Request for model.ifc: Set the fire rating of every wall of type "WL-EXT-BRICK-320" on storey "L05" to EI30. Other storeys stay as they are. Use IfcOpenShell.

First a look at what the model holds.

```python
import ifcopenshell
import ifcopenshell.util.element

model = ifcopenshell.open("model.ifc")
print(model.schema)
storey = next(s for s in model.by_type("IfcBuildingStorey") if s.Name == "L05")
walls = [e for e in ifcopenshell.util.element.get_decomposition(storey) if e.is_a("IfcWall")]
seen = {}
for e in walls:
    element_type = ifcopenshell.util.element.get_type(e)
    key = (element_type.Name if element_type != e and element_type else None, ifcopenshell.util.element.get_pset(e, "Pset_WallCommon", "FireRating"))
    seen[key] = seen.get(key, 0) + 1
for (name, value), count in sorted(seen.items(), key=str):
    print(count, "x", name, "|", value)
```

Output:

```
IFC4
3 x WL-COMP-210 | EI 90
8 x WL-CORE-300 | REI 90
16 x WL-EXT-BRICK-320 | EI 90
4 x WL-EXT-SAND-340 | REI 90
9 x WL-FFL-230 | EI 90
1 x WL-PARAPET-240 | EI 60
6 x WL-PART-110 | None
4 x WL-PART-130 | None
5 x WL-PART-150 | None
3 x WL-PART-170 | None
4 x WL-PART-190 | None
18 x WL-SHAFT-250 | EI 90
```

```python
import ifcopenshell
import ifcopenshell.api.pset
import ifcopenshell.util.element

model = ifcopenshell.open("model.ifc")

storey = next(s for s in model.by_type("IfcBuildingStorey") if s.Name == "L05")
walls = [e for e in ifcopenshell.util.element.get_decomposition(storey) if e.is_a("IfcWall")]

count = 0
for e in walls:
    element_type = ifcopenshell.util.element.get_type(e)
    if element_type in (None, e) or element_type.Name != "WL-EXT-BRICK-320":
        continue
    # add_pset returns the element's existing set when there is one.
    pset = ifcopenshell.api.pset.add_pset(model, product=e, name="Pset_WallCommon")
    ifcopenshell.api.pset.edit_pset(model, pset=pset, properties={"FireRating": "EI30"})
    count += 1

print(count, "walls updated")

model.write("model_edited.ifc")
```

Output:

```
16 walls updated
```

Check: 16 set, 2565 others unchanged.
